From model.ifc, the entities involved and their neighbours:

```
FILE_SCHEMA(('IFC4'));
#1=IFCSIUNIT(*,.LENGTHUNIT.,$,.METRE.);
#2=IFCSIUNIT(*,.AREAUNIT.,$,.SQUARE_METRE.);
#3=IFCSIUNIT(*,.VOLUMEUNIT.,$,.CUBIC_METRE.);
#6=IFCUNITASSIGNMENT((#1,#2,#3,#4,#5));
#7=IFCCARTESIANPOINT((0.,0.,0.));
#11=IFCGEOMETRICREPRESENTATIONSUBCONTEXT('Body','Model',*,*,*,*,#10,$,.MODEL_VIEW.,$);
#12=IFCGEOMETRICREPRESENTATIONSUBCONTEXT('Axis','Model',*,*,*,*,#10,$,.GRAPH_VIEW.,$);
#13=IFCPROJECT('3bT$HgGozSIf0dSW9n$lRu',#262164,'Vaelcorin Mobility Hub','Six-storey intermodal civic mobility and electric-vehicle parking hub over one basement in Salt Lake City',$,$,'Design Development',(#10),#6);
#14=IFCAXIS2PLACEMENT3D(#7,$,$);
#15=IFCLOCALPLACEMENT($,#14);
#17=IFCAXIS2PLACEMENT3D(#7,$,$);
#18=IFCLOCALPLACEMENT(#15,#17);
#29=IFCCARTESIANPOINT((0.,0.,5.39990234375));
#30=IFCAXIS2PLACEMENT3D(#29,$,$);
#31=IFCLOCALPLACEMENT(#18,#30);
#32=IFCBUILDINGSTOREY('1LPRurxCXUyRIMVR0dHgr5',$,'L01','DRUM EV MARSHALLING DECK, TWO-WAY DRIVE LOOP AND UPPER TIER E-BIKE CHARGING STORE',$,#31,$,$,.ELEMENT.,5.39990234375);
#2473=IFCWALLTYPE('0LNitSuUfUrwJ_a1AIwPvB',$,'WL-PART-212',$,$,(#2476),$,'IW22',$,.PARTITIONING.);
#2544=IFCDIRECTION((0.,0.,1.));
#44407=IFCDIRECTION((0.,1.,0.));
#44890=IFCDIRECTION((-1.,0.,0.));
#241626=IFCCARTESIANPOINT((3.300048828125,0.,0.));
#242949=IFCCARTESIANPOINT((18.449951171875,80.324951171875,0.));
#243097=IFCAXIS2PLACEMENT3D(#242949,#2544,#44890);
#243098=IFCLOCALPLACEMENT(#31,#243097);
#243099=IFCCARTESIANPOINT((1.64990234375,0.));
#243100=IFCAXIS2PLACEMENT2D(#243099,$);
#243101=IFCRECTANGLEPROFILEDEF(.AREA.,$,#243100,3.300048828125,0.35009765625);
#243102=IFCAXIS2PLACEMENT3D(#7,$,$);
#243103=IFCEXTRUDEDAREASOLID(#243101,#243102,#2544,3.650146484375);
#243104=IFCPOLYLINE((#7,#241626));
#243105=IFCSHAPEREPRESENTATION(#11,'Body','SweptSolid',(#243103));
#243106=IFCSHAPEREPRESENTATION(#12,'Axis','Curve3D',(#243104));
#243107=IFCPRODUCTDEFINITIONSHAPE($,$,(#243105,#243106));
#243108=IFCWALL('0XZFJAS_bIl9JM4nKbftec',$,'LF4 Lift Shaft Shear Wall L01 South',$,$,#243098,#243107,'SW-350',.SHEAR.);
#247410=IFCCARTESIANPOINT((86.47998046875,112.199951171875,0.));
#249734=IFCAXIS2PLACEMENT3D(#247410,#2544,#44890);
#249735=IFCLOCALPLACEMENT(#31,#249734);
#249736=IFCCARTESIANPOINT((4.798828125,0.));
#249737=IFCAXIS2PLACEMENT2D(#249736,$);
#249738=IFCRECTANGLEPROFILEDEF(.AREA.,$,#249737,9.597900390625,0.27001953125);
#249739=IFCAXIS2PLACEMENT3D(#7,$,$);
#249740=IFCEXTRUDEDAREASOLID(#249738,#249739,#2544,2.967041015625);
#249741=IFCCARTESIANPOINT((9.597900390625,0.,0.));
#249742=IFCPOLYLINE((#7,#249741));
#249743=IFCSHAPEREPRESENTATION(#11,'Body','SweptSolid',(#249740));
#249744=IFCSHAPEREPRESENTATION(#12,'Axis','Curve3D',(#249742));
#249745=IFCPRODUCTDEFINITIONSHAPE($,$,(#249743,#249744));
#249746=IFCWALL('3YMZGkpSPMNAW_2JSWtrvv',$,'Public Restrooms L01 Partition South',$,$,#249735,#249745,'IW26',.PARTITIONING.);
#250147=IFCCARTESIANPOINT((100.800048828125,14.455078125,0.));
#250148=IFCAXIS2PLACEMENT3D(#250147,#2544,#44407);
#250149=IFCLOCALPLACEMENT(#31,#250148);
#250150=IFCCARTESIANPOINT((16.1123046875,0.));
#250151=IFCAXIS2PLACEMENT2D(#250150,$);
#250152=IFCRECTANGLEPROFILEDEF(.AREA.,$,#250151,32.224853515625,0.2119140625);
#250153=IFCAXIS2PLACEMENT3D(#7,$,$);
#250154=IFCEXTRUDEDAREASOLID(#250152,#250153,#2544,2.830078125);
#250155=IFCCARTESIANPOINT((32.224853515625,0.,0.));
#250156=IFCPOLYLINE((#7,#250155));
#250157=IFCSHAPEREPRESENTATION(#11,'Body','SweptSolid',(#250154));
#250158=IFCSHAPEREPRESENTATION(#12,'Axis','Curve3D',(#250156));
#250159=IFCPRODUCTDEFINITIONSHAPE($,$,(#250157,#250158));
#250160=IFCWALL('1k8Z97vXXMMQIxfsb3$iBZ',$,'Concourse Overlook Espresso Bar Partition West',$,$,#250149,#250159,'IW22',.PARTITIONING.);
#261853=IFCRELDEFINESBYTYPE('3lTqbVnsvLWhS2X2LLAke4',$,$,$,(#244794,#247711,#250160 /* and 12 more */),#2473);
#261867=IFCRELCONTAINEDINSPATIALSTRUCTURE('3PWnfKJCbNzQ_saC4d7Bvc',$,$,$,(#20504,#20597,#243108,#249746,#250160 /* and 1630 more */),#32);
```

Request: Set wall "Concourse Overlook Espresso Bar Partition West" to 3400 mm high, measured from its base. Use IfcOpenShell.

```python
import ifcopenshell
import ifcopenshell.geom
import ifcopenshell.util.representation
import ifcopenshell.util.shape

model = ifcopenshell.open("model.ifc")
settings = ifcopenshell.geom.settings()


def volume(element):
    """Net volume in cubic metres, openings subtracted."""
    shape = ifcopenshell.geom.create_shape(settings, element)
    return ifcopenshell.util.shape.get_volume(shape.geometry)


wall = model.by_guid("1k8Z97vXXMMQIxfsb3$iBZ")
before = volume(wall)

body = ifcopenshell.util.representation.get_representation(wall, "Model", "Body")
solid = body.Items[0]
old_height = solid.Depth
solid.Depth = 3.4
after = volume(wall)

print(f"height {old_height:g} -> {solid.Depth:g}, volume {before:.3f} -> {after:.3f} m3")

model.write("model_rev.ifc")
```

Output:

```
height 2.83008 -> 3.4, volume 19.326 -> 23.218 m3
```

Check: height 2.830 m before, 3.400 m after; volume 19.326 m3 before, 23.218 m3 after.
